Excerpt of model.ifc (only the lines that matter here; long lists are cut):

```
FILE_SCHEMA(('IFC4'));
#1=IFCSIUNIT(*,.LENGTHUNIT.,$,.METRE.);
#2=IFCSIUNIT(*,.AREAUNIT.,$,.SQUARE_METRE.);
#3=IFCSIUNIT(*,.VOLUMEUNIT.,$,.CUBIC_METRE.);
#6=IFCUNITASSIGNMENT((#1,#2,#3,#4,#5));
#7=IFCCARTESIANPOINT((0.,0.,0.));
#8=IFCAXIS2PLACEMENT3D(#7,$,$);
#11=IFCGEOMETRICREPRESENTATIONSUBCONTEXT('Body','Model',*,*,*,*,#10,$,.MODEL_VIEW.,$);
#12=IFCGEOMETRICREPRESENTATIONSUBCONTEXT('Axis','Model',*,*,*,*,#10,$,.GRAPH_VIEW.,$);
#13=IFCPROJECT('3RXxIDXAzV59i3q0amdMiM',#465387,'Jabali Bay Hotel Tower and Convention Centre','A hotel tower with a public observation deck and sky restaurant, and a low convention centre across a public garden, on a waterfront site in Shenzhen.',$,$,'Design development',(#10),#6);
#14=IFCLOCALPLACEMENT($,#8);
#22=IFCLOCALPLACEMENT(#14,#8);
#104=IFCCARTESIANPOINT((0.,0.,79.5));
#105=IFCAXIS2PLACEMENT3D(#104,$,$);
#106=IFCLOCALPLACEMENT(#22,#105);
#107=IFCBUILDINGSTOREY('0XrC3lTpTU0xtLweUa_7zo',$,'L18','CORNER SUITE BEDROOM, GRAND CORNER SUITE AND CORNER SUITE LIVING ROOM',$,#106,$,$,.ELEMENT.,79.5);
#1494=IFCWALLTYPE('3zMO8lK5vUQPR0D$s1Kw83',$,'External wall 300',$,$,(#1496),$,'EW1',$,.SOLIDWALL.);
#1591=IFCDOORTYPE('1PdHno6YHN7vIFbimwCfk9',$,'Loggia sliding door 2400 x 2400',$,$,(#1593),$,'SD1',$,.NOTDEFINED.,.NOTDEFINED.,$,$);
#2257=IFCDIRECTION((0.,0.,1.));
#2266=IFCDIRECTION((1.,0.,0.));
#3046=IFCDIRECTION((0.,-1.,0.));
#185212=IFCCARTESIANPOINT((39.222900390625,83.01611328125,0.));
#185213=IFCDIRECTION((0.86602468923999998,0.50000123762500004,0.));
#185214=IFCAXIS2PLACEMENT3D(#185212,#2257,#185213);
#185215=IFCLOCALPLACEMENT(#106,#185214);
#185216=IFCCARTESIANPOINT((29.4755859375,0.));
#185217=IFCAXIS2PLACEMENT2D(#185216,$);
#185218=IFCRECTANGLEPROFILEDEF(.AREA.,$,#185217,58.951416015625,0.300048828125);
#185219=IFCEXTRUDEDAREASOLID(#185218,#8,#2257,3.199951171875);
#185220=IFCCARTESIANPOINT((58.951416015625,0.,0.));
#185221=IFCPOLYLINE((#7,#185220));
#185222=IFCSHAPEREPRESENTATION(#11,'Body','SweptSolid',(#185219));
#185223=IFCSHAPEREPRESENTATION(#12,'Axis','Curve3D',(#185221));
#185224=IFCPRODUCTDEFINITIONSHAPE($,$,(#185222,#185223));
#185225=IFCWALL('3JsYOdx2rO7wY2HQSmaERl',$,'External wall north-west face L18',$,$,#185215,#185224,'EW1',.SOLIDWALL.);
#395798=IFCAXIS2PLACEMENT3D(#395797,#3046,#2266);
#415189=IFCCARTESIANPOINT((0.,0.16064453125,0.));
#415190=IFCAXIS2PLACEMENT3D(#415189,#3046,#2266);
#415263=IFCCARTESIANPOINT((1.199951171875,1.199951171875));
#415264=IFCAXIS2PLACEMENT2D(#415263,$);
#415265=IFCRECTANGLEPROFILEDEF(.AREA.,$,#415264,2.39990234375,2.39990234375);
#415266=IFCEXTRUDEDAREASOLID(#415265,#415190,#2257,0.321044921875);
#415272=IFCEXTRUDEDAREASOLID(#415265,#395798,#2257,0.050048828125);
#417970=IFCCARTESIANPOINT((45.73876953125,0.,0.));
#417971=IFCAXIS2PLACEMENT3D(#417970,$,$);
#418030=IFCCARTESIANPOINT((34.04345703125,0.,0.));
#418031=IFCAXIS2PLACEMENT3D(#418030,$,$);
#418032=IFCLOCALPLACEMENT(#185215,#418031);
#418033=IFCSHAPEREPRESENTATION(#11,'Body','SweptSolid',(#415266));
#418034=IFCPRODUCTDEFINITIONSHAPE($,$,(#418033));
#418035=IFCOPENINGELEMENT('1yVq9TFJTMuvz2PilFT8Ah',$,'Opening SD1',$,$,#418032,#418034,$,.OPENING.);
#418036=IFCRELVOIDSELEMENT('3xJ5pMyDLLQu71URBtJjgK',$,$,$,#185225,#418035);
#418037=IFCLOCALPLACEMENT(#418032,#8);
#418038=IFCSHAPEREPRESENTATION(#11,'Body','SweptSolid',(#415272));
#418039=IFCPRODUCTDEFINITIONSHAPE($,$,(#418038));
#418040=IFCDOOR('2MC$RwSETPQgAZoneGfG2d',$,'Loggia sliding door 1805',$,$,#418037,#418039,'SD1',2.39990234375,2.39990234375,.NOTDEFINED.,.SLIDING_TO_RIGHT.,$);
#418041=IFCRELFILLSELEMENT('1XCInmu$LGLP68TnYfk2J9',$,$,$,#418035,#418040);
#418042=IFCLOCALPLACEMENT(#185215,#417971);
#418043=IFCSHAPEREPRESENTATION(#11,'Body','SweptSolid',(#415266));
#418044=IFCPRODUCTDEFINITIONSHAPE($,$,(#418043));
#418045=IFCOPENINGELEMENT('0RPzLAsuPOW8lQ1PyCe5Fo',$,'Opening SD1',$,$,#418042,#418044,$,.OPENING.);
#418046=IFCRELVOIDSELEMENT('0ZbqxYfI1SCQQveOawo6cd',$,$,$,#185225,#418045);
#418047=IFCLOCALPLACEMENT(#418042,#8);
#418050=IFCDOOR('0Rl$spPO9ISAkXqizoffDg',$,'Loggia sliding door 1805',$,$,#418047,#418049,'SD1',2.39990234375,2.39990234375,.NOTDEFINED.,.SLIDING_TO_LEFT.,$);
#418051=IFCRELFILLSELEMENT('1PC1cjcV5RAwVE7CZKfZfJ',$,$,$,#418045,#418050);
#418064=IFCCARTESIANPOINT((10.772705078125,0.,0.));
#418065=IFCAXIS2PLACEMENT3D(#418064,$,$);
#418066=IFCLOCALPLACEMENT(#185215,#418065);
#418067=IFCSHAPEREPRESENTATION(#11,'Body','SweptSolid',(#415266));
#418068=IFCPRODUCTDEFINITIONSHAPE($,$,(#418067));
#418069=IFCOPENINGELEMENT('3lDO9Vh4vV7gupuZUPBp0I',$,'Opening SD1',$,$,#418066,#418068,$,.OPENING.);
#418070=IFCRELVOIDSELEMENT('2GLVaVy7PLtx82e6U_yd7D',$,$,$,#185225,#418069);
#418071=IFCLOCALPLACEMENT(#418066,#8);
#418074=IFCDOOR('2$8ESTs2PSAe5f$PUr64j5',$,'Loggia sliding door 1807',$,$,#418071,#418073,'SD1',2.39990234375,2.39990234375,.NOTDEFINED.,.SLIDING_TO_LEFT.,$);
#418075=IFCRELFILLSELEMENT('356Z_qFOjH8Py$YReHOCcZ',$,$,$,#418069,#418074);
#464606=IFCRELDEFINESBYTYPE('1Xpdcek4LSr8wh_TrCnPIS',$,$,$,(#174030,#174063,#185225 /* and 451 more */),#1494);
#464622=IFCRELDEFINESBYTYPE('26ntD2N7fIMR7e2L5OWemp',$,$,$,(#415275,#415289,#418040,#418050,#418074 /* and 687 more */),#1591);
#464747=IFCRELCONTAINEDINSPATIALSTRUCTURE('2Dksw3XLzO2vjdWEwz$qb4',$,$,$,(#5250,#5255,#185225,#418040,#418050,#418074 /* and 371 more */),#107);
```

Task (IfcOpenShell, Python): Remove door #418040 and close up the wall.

```python
import ifcopenshell
import ifcopenshell.api.feature
import ifcopenshell.api.root
import ifcopenshell.geom
import ifcopenshell.util.shape

model = ifcopenshell.open("model.ifc")
settings = ifcopenshell.geom.settings()


def volume(element):
    """Net volume in cubic metres, openings subtracted."""
    shape = ifcopenshell.geom.create_shape(settings, element)
    return ifcopenshell.util.shape.get_volume(shape.geometry)


door = model.by_id(418040)
opening = door.FillsVoids[0].RelatingOpeningElement
wall = opening.VoidsElements[0].RelatingBuildingElement
before = volume(wall)

ifcopenshell.api.root.remove_product(model, product=door)
ifcopenshell.api.feature.remove_feature(model, feature=opening)

after = volume(wall)

print(f"wall volume {before:.3f} -> {after:.3f} m3")

model.write("model_edited.ifc")
```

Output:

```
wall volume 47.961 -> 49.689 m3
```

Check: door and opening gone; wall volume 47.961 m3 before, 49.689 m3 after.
